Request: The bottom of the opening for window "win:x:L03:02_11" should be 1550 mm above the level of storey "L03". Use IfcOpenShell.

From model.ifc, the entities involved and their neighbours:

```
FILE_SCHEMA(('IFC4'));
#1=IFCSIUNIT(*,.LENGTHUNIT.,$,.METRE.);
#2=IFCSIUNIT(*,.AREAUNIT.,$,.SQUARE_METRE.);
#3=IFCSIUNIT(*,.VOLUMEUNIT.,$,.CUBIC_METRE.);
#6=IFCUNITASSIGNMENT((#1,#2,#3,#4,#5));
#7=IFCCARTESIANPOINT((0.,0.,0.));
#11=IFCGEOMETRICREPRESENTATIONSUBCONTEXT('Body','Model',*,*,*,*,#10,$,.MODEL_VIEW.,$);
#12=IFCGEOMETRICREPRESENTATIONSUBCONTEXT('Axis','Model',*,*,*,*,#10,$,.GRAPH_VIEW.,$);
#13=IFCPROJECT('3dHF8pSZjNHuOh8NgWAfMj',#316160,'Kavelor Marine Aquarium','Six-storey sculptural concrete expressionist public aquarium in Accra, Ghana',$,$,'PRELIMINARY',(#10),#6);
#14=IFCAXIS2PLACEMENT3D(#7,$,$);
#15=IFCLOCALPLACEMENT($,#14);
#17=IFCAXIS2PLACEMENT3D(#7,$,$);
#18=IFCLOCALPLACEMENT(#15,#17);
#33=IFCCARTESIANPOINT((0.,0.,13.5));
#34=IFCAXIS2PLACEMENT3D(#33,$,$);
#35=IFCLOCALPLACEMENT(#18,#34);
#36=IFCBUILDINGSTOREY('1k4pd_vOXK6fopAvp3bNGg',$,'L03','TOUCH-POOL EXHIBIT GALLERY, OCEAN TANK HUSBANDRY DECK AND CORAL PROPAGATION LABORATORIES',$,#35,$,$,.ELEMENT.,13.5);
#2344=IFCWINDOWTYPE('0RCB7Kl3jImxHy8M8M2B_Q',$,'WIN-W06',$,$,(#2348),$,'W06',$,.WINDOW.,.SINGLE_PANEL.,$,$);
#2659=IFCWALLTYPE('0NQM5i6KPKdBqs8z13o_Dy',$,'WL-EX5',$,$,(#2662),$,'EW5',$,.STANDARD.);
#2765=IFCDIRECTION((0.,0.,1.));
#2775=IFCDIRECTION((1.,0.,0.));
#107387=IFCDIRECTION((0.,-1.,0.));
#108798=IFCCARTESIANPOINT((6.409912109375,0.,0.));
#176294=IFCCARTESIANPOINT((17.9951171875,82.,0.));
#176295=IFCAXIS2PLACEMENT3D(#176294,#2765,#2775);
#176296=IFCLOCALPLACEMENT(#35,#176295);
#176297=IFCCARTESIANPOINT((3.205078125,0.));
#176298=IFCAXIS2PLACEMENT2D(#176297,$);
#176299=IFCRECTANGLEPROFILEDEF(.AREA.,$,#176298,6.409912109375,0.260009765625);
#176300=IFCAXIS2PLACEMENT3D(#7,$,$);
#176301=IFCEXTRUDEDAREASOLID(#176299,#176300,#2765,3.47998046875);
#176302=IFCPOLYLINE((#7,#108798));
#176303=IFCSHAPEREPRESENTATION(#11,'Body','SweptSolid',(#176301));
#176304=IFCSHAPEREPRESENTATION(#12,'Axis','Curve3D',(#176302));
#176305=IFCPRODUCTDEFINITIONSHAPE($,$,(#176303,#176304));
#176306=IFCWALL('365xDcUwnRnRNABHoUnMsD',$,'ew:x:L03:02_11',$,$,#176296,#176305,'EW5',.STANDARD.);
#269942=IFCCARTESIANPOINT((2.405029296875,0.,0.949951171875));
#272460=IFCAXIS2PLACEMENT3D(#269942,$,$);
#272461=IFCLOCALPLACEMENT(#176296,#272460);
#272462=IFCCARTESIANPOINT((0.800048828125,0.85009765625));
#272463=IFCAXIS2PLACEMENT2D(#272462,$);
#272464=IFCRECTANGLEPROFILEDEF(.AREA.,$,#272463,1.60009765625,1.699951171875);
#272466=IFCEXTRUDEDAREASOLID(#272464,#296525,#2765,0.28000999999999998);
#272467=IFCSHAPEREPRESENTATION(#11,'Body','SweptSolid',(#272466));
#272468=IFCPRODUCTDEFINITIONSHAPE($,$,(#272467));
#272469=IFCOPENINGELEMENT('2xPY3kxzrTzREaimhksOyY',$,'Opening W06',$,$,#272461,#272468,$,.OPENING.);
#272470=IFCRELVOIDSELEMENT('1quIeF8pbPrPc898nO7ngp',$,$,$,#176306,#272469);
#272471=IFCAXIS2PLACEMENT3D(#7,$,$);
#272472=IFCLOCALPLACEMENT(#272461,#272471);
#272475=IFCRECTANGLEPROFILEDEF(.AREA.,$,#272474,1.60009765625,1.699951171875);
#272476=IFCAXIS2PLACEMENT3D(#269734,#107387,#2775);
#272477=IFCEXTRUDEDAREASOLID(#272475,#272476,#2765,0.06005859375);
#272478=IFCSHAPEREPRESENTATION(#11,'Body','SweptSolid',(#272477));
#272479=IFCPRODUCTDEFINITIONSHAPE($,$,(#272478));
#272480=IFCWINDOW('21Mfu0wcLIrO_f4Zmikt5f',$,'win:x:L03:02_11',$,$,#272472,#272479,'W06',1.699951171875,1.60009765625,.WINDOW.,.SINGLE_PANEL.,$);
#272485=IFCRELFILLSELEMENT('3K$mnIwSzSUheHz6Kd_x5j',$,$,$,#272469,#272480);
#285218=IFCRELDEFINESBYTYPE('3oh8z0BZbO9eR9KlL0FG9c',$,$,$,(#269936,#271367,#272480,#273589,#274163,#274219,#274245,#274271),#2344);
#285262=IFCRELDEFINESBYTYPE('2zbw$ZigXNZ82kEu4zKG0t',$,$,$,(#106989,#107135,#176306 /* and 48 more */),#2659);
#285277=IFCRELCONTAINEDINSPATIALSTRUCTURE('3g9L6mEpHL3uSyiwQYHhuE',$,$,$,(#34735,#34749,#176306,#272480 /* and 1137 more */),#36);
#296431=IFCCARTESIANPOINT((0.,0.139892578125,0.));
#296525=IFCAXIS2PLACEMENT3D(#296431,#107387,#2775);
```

```python
import numpy as np
import ifcopenshell
import ifcopenshell.api.geometry
import ifcopenshell.geom
import ifcopenshell.util.element
import ifcopenshell.util.placement
import ifcopenshell.util.shape
import ifcopenshell.util.unit

model = ifcopenshell.open("model.ifc")
unit_scale = ifcopenshell.util.unit.calculate_unit_scale(model)

window = model.by_guid("21Mfu0wcLIrO_f4Zmikt5f")
opening = window.FillsVoids[0].RelatingOpeningElement
storey = ifcopenshell.util.element.get_container(window, ifc_class="IfcBuildingStorey")
level = ifcopenshell.util.placement.get_local_placement(storey.ObjectPlacement)[2, 3]

# The opening's origin need not be at the sill, so measure its lowest point.
shape = ifcopenshell.geom.create_shape(ifcopenshell.geom.settings(), opening)
bottom = ifcopenshell.util.shape.get_shape_bottom_elevation(shape, shape.geometry) / unit_scale
dz = level + 1.55 - bottom

shift = np.array([0.0, 0.0, dz])
# The window is placed relative to its opening, so it follows when the opening moves.
matrix = ifcopenshell.util.placement.get_local_placement(opening.ObjectPlacement)
matrix[:3, 3] += shift
ifcopenshell.api.geometry.edit_object_placement(
    model, product=opening, matrix=matrix, is_si=False, should_transform_children=True
)

print(f"moved by {dz * unit_scale:+.3f} m")

model.write("model_edited.ifc")
```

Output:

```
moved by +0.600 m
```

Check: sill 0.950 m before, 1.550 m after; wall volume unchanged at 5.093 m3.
